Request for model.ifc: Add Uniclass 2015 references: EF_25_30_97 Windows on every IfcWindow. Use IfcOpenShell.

First a look at what the model holds.

```python
import ifcopenshell

model = ifcopenshell.open("model.ifc")
print(model.schema)
print("classifications:", [c.Name for c in model.by_type("IfcClassification")])
for ifc_class in ("IfcDoor", "IfcRoof", "IfcStair", "IfcWall", "IfcWindow"):
    print(ifc_class, len(model.by_type(ifc_class)))
```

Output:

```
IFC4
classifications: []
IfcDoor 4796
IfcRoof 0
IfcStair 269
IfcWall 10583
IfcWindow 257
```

```python
import ifcopenshell
import ifcopenshell.api.classification

model = ifcopenshell.open("model.ifc")

system = ifcopenshell.api.classification.add_classification(model, classification="Uniclass 2015")

codes = {
    "IfcWindow": ("EF_25_30_97", "Windows"),
}
for ifc_class, (code, name) in codes.items():
    products = model.by_type(ifc_class)
    ifcopenshell.api.classification.add_reference(
        model, products=products, classification=system, identification=code, name=name
    )
    print(code, len(products))

model.write("model_edited.ifc")
```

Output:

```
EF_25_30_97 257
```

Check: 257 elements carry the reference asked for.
